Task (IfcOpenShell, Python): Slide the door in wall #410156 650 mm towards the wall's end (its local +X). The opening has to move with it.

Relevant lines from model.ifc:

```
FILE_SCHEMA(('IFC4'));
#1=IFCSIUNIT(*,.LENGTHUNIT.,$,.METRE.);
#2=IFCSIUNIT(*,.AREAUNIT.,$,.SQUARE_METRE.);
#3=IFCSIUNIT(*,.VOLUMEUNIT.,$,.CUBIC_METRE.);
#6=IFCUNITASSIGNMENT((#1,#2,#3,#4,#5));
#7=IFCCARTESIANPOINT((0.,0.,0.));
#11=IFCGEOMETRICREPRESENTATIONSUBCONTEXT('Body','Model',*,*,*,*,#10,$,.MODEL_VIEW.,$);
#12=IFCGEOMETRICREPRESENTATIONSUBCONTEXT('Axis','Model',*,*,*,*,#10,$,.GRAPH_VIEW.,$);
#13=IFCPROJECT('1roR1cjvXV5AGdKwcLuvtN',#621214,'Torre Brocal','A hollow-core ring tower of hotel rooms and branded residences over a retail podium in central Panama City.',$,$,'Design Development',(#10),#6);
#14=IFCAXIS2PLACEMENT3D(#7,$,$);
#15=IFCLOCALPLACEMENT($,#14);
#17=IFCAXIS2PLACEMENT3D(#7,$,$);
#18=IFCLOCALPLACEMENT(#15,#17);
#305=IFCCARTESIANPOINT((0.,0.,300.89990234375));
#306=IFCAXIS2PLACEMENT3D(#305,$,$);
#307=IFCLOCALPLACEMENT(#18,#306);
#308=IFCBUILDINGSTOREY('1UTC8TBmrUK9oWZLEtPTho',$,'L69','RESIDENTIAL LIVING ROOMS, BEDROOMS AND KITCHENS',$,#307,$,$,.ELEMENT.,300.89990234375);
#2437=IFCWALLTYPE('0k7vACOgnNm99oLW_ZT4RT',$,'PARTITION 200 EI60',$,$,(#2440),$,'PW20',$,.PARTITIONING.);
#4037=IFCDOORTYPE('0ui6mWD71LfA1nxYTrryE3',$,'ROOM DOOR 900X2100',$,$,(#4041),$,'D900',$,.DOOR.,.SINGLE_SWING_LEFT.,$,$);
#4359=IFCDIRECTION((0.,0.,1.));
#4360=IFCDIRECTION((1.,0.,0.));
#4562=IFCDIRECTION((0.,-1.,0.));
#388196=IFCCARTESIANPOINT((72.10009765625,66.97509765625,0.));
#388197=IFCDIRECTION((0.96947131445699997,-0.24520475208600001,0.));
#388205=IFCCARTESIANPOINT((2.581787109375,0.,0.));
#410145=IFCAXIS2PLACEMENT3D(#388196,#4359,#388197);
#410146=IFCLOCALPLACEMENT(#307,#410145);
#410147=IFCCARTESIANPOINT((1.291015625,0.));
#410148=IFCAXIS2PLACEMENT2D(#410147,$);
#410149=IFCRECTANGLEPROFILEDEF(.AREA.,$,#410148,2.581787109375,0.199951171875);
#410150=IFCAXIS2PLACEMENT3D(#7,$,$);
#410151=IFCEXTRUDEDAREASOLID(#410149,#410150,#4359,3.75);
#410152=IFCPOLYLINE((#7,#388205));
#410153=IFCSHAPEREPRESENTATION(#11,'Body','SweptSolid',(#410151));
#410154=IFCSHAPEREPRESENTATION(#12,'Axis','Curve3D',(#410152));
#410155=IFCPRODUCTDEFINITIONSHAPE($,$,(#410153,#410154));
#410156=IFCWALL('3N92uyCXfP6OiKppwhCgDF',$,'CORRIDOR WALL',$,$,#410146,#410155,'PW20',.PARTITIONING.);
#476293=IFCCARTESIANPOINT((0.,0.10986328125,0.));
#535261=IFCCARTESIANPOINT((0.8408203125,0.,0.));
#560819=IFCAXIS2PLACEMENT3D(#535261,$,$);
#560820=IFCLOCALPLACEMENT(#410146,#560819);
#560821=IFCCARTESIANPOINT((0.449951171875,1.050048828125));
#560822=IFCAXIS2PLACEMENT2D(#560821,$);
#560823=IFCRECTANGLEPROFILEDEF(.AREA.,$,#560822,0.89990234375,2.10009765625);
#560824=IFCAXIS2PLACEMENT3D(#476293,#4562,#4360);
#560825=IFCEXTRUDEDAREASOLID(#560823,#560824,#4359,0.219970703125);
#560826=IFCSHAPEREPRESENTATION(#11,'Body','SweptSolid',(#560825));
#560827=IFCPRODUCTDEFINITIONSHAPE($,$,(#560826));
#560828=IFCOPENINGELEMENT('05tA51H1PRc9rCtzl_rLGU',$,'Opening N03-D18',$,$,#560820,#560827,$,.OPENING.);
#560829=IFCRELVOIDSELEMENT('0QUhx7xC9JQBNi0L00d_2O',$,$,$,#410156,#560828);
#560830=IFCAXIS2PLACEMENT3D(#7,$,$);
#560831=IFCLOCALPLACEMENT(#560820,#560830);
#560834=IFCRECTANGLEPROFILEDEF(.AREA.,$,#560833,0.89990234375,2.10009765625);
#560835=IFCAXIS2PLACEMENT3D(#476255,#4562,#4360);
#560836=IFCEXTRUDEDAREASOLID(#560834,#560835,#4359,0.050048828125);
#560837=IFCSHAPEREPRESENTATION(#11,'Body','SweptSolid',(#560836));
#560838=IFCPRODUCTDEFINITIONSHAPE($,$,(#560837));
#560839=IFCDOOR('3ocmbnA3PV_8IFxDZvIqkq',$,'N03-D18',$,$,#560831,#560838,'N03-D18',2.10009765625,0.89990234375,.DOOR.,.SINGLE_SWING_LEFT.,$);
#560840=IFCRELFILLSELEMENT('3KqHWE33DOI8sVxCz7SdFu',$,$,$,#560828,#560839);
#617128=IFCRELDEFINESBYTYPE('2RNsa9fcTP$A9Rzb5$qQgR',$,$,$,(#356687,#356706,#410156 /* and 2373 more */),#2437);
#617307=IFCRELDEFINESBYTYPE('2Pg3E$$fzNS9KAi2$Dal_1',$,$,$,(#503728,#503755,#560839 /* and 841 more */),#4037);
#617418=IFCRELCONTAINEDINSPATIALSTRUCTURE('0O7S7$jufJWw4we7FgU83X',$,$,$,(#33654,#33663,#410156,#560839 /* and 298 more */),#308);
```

```python
import ifcopenshell
import ifcopenshell.api.geometry
import ifcopenshell.util.placement
import ifcopenshell.util.unit

model = ifcopenshell.open("model.ifc")
unit_scale = ifcopenshell.util.unit.calculate_unit_scale(model)

door = model.by_id(560839)
opening = door.FillsVoids[0].RelatingOpeningElement
wall = opening.VoidsElements[0].RelatingBuildingElement

wall_matrix = ifcopenshell.util.placement.get_local_placement(wall.ObjectPlacement)
shift = wall_matrix[:3, 0] * 0.65 / unit_scale
before = ifcopenshell.util.placement.get_local_placement(door.ObjectPlacement)[:3, 3].copy()

# The door is placed relative to its opening, so it follows when the opening moves.
matrix = ifcopenshell.util.placement.get_local_placement(opening.ObjectPlacement)
matrix[:3, 3] += shift
ifcopenshell.api.geometry.edit_object_placement(
    model, product=opening, matrix=matrix, is_si=False, should_transform_children=True
)

after = ifcopenshell.util.placement.get_local_placement(door.ObjectPlacement)[:3, 3]
print("door moved by", (after - before).round(3) + 0.0)

model.write("model_v2.ifc")
```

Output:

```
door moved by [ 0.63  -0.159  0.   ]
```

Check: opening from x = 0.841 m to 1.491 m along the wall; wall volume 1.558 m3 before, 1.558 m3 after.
